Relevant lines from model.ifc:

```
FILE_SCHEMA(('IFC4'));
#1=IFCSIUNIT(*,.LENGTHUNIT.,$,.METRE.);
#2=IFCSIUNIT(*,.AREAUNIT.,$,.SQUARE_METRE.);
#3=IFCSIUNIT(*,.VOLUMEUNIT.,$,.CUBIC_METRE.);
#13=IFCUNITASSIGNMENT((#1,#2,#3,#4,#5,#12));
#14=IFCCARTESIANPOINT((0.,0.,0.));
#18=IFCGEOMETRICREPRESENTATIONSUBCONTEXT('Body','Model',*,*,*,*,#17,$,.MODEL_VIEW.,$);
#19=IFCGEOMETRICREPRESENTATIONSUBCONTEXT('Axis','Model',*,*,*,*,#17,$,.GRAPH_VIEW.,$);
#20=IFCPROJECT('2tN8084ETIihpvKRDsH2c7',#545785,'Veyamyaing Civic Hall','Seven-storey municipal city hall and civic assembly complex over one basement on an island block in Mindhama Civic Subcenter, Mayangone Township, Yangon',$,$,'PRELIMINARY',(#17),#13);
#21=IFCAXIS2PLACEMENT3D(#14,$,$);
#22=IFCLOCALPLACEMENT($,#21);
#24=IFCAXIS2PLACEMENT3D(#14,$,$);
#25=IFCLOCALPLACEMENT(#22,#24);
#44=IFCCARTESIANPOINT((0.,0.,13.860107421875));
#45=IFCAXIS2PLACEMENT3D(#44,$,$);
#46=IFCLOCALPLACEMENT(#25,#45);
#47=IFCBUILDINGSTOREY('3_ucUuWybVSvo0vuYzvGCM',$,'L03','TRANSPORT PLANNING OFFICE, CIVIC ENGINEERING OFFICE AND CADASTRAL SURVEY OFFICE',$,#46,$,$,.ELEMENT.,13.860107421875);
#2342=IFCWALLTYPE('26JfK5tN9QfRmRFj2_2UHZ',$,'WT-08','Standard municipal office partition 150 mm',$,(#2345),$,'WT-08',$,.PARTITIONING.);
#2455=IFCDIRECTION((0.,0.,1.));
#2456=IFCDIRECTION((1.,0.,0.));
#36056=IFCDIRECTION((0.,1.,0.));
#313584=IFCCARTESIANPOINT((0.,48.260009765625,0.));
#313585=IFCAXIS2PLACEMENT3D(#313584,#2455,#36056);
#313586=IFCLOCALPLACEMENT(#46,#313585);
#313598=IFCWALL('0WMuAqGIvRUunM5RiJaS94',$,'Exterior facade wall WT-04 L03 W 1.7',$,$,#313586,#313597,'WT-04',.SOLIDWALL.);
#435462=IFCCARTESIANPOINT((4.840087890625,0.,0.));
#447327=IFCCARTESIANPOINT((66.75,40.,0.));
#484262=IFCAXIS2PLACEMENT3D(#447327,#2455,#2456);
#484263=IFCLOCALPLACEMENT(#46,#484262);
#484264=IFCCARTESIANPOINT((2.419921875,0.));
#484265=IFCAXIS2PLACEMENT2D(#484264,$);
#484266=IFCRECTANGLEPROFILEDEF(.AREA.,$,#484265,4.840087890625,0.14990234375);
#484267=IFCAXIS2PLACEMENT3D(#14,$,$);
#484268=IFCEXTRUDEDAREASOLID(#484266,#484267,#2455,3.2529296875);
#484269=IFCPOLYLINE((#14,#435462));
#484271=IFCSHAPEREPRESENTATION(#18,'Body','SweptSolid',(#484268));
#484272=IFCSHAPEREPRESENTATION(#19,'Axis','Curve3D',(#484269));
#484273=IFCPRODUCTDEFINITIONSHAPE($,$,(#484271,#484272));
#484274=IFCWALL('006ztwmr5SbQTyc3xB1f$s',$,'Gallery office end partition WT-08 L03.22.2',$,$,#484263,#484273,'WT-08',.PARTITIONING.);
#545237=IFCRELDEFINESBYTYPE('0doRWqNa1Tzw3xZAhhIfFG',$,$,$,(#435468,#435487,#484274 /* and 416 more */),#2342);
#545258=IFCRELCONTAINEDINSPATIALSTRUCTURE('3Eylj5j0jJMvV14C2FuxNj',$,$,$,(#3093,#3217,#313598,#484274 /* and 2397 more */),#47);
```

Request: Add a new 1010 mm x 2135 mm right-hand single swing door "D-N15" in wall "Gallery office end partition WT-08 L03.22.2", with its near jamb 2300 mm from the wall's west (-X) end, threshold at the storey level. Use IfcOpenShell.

```python
import numpy as np
import ifcopenshell
import ifcopenshell.api.feature
import ifcopenshell.api.geometry
import ifcopenshell.api.root
import ifcopenshell.api.spatial
import ifcopenshell.geom
import ifcopenshell.util.element
import ifcopenshell.util.placement
import ifcopenshell.util.representation
import ifcopenshell.util.shape
import ifcopenshell.util.unit

model = ifcopenshell.open("model.ifc")
unit_scale = ifcopenshell.util.unit.calculate_unit_scale(model)
settings = ifcopenshell.geom.settings()


def volume(element):
    """Net volume in cubic metres, openings subtracted."""
    shape = ifcopenshell.geom.create_shape(settings, element)
    return ifcopenshell.util.shape.get_volume(shape.geometry)


wall = model.by_guid("006ztwmr5SbQTyc3xB1f$s")
storey = ifcopenshell.util.element.get_container(wall, ifc_class="IfcBuildingStorey")
context = ifcopenshell.util.representation.get_context(model, "Model", "Body", "MODEL_VIEW")
before = volume(wall)

width, height, from_end, sill = 1.01, 2.135, 2.3, 0.0  # metres

# The wall runs along its own X axis, and the end named is its -X end.
wall_shape = ifcopenshell.geom.create_shape(settings, wall)
x, y, z = ifcopenshell.util.shape.get_vertices(wall_shape.geometry).T
start = x.min() + from_end
face, thickness = float(y.min()), float(y.max() - y.min())
wall_matrix = ifcopenshell.util.placement.get_local_placement(wall.ObjectPlacement)
level = ifcopenshell.util.placement.get_local_placement(storey.ObjectPlacement)[2, 3]


def in_wall(x, y):
    """Placement at x, y metres in the wall's axes, at sill height."""
    matrix = wall_matrix.copy()
    matrix[:, 3] = wall_matrix @ np.array([x / unit_scale, y / unit_scale, 0.0, 1.0])
    matrix[2, 3] = level + sill / unit_scale
    return matrix


# Opening: a box that overshoots both wall faces by 50 mm.
opening = ifcopenshell.api.root.create_entity(model, ifc_class="IfcOpeningElement", predefined_type="OPENING")
box = ifcopenshell.api.geometry.add_wall_representation(
    model, context=context, length=width, height=height, thickness=thickness + 0.1
)
ifcopenshell.api.geometry.assign_representation(model, product=opening, representation=box)
ifcopenshell.api.geometry.edit_object_placement(model, product=opening, matrix=in_wall(start, face - 0.05), is_si=False)
ifcopenshell.api.feature.add_feature(model, feature=opening, element=wall)

door = ifcopenshell.api.root.create_entity(model, ifc_class="IfcDoor", name="D-N15", predefined_type="DOOR")
door.OverallWidth, door.OverallHeight = width / unit_scale, height / unit_scale
door.OperationType = "SINGLE_SWING_RIGHT"
body = ifcopenshell.api.geometry.add_door_representation(
    model,
    context=context,
    overall_width=door.OverallWidth,
    overall_height=door.OverallHeight,
    operation_type="SINGLE_SWING_RIGHT",
    lining_properties={"LiningDepth": thickness / unit_scale, "ThresholdDepth": thickness / unit_scale},
)
ifcopenshell.api.geometry.assign_representation(model, product=door, representation=body)
ifcopenshell.api.spatial.assign_container(model, products=[door], relating_structure=storey)
ifcopenshell.api.feature.add_filling(model, opening=opening, element=door)

# The lining spans the wall, so the door starts at the wall face.
ifcopenshell.api.geometry.edit_object_placement(model, product=door, matrix=in_wall(start, face), is_si=False)

after = volume(wall)

print(f"wall volume {before:.3f} -> {after:.3f} m3")

model.write("model-out.ifc")
```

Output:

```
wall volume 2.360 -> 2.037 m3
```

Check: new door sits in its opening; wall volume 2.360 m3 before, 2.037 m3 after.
